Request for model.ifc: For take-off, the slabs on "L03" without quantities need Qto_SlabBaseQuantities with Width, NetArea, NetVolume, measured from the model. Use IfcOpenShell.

First a look at what the model holds.

```python
import ifcopenshell
import ifcopenshell.util.element
import ifcopenshell.util.unit

model = ifcopenshell.open("model.ifc")
print(model.schema)
for unit_type in ("LENGTHUNIT", "AREAUNIT", "VOLUMEUNIT"):
    print(unit_type, ifcopenshell.util.unit.calculate_unit_scale(model, unit_type))
storey = next(s for s in model.by_type("IfcBuildingStorey") if s.Name == "L03")
slabs = [e for e in ifcopenshell.util.element.get_decomposition(storey) if e.is_a("IfcSlab")]
for e in sorted(slabs, key=lambda e: e.id()):
    print(e.id(), e.is_a(), e.Name, list(ifcopenshell.util.element.get_psets(e, qtos_only=True)), sep=" | ")
```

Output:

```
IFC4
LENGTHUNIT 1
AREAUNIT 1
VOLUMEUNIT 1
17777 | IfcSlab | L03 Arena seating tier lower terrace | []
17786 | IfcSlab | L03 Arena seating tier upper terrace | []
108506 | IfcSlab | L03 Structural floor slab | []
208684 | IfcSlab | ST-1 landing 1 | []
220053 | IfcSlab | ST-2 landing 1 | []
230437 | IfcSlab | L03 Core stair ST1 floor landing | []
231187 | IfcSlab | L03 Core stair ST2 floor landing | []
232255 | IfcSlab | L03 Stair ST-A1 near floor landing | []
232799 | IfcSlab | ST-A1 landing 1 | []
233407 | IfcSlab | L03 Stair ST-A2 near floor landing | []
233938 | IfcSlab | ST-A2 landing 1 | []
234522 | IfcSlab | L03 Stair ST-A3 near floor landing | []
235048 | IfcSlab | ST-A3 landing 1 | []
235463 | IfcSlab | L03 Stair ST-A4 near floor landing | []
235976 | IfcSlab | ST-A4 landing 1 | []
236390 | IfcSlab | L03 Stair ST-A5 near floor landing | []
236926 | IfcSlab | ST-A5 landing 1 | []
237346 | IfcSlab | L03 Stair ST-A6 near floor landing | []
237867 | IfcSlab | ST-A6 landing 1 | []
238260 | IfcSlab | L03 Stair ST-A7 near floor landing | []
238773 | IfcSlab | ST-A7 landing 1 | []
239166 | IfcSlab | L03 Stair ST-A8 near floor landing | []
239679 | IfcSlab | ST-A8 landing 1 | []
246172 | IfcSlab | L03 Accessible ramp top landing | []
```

```python
import ifcopenshell
import ifcopenshell.api.pset
import ifcopenshell.geom
import ifcopenshell.util.element
import ifcopenshell.util.shape
import ifcopenshell.util.unit

model = ifcopenshell.open("model.ifc")
unit_scale = ifcopenshell.util.unit.calculate_unit_scale(model)
area_scale = ifcopenshell.util.unit.calculate_unit_scale(model, "AREAUNIT")
volume_scale = ifcopenshell.util.unit.calculate_unit_scale(model, "VOLUMEUNIT")
settings = ifcopenshell.geom.settings()

storey = next(s for s in model.by_type("IfcBuildingStorey") if s.Name == "L03")
slabs = [e for e in ifcopenshell.util.element.get_decomposition(storey) if e.is_a("IfcSlab")]

for e in sorted(slabs, key=lambda e: e.id()):
    if ifcopenshell.util.element.get_psets(e, qtos_only=True, should_inherit=False):
        continue
    # Geometry comes back in metres, in the element's own axes.
    shape = ifcopenshell.geom.create_shape(settings, e)
    values = {
        "Width": ifcopenshell.util.shape.get_z(shape.geometry) / unit_scale,
        "NetArea": ifcopenshell.util.shape.get_footprint_area(shape.geometry) / area_scale,
        "NetVolume": ifcopenshell.util.shape.get_volume(shape.geometry) / volume_scale,
    }
    qto = ifcopenshell.api.pset.add_qto(model, product=e, name="Qto_SlabBaseQuantities")
    ifcopenshell.api.pset.edit_qto(model, qto=qto, properties=values)
    print(e.id(), {k: round(v, 3) for k, v in values.items()})

model.write("model_updated.ifc")
```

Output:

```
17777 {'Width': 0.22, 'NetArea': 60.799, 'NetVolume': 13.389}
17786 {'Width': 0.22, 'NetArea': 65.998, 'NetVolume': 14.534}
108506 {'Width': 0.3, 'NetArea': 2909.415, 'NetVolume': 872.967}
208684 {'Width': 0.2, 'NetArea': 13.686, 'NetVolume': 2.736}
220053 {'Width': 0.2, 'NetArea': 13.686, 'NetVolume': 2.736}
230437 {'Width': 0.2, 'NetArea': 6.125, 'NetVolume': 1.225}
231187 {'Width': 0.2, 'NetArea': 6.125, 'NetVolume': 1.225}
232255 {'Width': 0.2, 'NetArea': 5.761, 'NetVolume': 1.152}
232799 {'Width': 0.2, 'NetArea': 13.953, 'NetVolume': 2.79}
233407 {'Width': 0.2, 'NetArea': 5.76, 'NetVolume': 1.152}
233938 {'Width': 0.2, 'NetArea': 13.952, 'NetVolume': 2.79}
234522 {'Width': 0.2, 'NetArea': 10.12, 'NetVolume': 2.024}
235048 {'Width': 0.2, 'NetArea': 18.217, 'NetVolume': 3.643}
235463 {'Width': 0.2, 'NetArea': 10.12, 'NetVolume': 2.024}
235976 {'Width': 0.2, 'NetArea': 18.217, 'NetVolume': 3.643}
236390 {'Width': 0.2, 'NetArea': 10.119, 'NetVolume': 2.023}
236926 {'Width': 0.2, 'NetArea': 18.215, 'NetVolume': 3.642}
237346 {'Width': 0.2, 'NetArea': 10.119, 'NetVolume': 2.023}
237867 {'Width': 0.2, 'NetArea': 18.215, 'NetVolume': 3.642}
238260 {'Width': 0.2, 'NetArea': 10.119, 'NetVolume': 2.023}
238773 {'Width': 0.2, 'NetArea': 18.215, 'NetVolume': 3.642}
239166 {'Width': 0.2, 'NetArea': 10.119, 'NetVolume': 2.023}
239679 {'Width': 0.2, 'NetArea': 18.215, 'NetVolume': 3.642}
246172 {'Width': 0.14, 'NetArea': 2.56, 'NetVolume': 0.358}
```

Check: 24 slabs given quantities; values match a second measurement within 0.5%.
